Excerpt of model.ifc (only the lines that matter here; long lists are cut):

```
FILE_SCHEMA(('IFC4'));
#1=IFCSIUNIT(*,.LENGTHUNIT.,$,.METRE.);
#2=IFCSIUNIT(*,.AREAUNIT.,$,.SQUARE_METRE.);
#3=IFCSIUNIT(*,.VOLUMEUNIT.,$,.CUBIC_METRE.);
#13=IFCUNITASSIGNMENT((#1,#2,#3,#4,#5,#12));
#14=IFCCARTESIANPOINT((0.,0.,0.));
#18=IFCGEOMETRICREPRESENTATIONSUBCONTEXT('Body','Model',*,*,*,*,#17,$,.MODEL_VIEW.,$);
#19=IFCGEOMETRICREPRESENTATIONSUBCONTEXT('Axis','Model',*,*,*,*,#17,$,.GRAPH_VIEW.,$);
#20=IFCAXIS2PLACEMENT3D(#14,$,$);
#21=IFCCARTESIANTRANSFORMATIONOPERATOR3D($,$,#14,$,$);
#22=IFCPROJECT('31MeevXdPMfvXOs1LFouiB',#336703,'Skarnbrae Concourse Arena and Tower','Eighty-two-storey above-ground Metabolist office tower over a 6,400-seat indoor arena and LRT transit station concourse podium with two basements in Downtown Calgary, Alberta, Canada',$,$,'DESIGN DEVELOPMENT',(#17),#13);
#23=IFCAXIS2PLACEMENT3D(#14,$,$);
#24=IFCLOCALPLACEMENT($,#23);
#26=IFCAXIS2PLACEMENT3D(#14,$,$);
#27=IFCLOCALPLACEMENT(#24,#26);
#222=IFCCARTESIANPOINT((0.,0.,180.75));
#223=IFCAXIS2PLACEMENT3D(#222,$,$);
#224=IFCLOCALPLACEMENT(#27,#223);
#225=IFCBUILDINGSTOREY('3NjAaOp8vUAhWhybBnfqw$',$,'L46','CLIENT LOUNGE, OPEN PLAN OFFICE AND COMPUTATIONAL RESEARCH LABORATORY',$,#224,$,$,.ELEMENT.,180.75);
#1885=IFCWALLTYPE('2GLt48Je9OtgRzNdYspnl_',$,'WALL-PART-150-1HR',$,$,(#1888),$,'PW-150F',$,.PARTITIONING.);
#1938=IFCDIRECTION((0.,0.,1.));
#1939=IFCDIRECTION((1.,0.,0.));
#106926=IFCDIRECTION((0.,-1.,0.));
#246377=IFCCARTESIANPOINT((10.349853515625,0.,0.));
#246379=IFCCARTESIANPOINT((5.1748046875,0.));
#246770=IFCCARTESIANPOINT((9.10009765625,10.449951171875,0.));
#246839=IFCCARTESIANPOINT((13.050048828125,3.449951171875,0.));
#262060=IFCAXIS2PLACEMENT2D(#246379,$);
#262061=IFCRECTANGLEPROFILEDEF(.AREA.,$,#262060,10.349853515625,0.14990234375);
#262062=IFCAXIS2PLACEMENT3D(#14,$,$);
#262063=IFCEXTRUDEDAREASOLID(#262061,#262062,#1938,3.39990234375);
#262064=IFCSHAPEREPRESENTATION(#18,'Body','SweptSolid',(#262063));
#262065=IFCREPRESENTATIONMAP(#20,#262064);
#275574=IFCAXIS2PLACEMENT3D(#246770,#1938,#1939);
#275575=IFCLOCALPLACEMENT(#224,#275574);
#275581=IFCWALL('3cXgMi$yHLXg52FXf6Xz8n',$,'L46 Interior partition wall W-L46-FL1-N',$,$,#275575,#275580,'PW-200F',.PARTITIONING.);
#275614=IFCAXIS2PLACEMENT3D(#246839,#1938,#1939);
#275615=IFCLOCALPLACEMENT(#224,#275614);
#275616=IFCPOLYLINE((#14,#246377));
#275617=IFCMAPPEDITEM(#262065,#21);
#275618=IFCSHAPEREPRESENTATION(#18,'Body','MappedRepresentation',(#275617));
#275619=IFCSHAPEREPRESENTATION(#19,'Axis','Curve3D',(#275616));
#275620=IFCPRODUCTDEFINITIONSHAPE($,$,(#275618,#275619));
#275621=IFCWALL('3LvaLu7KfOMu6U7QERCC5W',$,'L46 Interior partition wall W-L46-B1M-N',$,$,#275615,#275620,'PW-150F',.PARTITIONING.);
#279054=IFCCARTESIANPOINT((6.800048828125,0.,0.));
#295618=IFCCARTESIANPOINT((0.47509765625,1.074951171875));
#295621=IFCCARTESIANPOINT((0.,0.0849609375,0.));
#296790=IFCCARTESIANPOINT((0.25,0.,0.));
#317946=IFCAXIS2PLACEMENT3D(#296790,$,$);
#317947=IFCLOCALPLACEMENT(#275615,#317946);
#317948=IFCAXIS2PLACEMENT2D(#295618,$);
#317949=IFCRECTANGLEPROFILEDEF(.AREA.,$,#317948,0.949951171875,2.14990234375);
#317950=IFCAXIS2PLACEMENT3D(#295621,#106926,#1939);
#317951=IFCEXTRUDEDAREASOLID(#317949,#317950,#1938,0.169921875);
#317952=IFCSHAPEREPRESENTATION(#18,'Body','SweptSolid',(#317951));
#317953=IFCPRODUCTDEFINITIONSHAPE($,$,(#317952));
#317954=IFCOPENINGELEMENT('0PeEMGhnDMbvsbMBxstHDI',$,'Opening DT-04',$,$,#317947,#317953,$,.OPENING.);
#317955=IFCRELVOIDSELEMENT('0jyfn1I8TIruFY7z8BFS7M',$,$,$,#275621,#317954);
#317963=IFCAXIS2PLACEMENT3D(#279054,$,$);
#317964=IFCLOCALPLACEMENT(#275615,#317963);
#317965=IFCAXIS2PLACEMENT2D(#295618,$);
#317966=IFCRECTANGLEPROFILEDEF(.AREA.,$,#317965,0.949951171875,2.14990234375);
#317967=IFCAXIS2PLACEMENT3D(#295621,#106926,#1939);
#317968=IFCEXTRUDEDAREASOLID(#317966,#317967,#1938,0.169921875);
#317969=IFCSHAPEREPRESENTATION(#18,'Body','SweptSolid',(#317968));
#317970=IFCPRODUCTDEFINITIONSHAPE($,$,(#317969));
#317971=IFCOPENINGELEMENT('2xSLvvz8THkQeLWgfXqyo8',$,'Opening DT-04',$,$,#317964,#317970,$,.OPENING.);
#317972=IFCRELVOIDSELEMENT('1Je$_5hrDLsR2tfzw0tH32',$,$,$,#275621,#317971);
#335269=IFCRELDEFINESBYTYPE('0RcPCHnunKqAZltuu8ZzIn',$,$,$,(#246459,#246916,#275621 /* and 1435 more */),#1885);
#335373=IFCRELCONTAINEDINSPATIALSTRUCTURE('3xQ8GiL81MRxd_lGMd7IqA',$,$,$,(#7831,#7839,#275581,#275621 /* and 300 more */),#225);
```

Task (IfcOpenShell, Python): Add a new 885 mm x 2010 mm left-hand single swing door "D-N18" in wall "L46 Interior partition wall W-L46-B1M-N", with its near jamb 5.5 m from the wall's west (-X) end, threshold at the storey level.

```python
import numpy as np
import ifcopenshell
import ifcopenshell.api.feature
import ifcopenshell.api.geometry
import ifcopenshell.api.root
import ifcopenshell.api.spatial
import ifcopenshell.geom
import ifcopenshell.util.element
import ifcopenshell.util.placement
import ifcopenshell.util.representation
import ifcopenshell.util.shape
import ifcopenshell.util.unit

model = ifcopenshell.open("model.ifc")
unit_scale = ifcopenshell.util.unit.calculate_unit_scale(model)
settings = ifcopenshell.geom.settings()


def volume(element):
    """Net volume in cubic metres, openings subtracted."""
    shape = ifcopenshell.geom.create_shape(settings, element)
    return ifcopenshell.util.shape.get_volume(shape.geometry)


wall = model.by_guid("3LvaLu7KfOMu6U7QERCC5W")
storey = ifcopenshell.util.element.get_container(wall, ifc_class="IfcBuildingStorey")
context = ifcopenshell.util.representation.get_context(model, "Model", "Body", "MODEL_VIEW")
before = volume(wall)

width, height, from_end, sill = 0.885, 2.01, 5.5, 0.0  # metres

# The wall runs along its own X axis, and the end named is its -X end.
wall_shape = ifcopenshell.geom.create_shape(settings, wall)
x, y, z = ifcopenshell.util.shape.get_vertices(wall_shape.geometry).T
start = x.min() + from_end
face, thickness = float(y.min()), float(y.max() - y.min())
wall_matrix = ifcopenshell.util.placement.get_local_placement(wall.ObjectPlacement)
level = ifcopenshell.util.placement.get_local_placement(storey.ObjectPlacement)[2, 3]


def in_wall(x, y):
    """Placement at x, y metres in the wall's axes, at sill height."""
    matrix = wall_matrix.copy()
    matrix[:, 3] = wall_matrix @ np.array([x / unit_scale, y / unit_scale, 0.0, 1.0])
    matrix[2, 3] = level + sill / unit_scale
    return matrix


# Opening: a box that overshoots both wall faces by 50 mm.
opening = ifcopenshell.api.root.create_entity(model, ifc_class="IfcOpeningElement", predefined_type="OPENING")
box = ifcopenshell.api.geometry.add_wall_representation(
    model, context=context, length=width, height=height, thickness=thickness + 0.1
)
ifcopenshell.api.geometry.assign_representation(model, product=opening, representation=box)
ifcopenshell.api.geometry.edit_object_placement(model, product=opening, matrix=in_wall(start, face - 0.05), is_si=False)
ifcopenshell.api.feature.add_feature(model, feature=opening, element=wall)

door = ifcopenshell.api.root.create_entity(model, ifc_class="IfcDoor", name="D-N18", predefined_type="DOOR")
door.OverallWidth, door.OverallHeight = width / unit_scale, height / unit_scale
door.OperationType = "SINGLE_SWING_LEFT"
body = ifcopenshell.api.geometry.add_door_representation(
    model,
    context=context,
    overall_width=door.OverallWidth,
    overall_height=door.OverallHeight,
    operation_type="SINGLE_SWING_LEFT",
    lining_properties={"LiningDepth": thickness / unit_scale, "ThresholdDepth": thickness / unit_scale},
)
ifcopenshell.api.geometry.assign_representation(model, product=door, representation=body)
ifcopenshell.api.spatial.assign_container(model, products=[door], relating_structure=storey)
ifcopenshell.api.feature.add_filling(model, opening=opening, element=door)

# The lining spans the wall, so the door starts at the wall face.
ifcopenshell.api.geometry.edit_object_placement(model, product=door, matrix=in_wall(start, face), is_si=False)

after = volume(wall)

print(f"wall volume {before:.3f} -> {after:.3f} m3")

model.write("model-out.ifc")
```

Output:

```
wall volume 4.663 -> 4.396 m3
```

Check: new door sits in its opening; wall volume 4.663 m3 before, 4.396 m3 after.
